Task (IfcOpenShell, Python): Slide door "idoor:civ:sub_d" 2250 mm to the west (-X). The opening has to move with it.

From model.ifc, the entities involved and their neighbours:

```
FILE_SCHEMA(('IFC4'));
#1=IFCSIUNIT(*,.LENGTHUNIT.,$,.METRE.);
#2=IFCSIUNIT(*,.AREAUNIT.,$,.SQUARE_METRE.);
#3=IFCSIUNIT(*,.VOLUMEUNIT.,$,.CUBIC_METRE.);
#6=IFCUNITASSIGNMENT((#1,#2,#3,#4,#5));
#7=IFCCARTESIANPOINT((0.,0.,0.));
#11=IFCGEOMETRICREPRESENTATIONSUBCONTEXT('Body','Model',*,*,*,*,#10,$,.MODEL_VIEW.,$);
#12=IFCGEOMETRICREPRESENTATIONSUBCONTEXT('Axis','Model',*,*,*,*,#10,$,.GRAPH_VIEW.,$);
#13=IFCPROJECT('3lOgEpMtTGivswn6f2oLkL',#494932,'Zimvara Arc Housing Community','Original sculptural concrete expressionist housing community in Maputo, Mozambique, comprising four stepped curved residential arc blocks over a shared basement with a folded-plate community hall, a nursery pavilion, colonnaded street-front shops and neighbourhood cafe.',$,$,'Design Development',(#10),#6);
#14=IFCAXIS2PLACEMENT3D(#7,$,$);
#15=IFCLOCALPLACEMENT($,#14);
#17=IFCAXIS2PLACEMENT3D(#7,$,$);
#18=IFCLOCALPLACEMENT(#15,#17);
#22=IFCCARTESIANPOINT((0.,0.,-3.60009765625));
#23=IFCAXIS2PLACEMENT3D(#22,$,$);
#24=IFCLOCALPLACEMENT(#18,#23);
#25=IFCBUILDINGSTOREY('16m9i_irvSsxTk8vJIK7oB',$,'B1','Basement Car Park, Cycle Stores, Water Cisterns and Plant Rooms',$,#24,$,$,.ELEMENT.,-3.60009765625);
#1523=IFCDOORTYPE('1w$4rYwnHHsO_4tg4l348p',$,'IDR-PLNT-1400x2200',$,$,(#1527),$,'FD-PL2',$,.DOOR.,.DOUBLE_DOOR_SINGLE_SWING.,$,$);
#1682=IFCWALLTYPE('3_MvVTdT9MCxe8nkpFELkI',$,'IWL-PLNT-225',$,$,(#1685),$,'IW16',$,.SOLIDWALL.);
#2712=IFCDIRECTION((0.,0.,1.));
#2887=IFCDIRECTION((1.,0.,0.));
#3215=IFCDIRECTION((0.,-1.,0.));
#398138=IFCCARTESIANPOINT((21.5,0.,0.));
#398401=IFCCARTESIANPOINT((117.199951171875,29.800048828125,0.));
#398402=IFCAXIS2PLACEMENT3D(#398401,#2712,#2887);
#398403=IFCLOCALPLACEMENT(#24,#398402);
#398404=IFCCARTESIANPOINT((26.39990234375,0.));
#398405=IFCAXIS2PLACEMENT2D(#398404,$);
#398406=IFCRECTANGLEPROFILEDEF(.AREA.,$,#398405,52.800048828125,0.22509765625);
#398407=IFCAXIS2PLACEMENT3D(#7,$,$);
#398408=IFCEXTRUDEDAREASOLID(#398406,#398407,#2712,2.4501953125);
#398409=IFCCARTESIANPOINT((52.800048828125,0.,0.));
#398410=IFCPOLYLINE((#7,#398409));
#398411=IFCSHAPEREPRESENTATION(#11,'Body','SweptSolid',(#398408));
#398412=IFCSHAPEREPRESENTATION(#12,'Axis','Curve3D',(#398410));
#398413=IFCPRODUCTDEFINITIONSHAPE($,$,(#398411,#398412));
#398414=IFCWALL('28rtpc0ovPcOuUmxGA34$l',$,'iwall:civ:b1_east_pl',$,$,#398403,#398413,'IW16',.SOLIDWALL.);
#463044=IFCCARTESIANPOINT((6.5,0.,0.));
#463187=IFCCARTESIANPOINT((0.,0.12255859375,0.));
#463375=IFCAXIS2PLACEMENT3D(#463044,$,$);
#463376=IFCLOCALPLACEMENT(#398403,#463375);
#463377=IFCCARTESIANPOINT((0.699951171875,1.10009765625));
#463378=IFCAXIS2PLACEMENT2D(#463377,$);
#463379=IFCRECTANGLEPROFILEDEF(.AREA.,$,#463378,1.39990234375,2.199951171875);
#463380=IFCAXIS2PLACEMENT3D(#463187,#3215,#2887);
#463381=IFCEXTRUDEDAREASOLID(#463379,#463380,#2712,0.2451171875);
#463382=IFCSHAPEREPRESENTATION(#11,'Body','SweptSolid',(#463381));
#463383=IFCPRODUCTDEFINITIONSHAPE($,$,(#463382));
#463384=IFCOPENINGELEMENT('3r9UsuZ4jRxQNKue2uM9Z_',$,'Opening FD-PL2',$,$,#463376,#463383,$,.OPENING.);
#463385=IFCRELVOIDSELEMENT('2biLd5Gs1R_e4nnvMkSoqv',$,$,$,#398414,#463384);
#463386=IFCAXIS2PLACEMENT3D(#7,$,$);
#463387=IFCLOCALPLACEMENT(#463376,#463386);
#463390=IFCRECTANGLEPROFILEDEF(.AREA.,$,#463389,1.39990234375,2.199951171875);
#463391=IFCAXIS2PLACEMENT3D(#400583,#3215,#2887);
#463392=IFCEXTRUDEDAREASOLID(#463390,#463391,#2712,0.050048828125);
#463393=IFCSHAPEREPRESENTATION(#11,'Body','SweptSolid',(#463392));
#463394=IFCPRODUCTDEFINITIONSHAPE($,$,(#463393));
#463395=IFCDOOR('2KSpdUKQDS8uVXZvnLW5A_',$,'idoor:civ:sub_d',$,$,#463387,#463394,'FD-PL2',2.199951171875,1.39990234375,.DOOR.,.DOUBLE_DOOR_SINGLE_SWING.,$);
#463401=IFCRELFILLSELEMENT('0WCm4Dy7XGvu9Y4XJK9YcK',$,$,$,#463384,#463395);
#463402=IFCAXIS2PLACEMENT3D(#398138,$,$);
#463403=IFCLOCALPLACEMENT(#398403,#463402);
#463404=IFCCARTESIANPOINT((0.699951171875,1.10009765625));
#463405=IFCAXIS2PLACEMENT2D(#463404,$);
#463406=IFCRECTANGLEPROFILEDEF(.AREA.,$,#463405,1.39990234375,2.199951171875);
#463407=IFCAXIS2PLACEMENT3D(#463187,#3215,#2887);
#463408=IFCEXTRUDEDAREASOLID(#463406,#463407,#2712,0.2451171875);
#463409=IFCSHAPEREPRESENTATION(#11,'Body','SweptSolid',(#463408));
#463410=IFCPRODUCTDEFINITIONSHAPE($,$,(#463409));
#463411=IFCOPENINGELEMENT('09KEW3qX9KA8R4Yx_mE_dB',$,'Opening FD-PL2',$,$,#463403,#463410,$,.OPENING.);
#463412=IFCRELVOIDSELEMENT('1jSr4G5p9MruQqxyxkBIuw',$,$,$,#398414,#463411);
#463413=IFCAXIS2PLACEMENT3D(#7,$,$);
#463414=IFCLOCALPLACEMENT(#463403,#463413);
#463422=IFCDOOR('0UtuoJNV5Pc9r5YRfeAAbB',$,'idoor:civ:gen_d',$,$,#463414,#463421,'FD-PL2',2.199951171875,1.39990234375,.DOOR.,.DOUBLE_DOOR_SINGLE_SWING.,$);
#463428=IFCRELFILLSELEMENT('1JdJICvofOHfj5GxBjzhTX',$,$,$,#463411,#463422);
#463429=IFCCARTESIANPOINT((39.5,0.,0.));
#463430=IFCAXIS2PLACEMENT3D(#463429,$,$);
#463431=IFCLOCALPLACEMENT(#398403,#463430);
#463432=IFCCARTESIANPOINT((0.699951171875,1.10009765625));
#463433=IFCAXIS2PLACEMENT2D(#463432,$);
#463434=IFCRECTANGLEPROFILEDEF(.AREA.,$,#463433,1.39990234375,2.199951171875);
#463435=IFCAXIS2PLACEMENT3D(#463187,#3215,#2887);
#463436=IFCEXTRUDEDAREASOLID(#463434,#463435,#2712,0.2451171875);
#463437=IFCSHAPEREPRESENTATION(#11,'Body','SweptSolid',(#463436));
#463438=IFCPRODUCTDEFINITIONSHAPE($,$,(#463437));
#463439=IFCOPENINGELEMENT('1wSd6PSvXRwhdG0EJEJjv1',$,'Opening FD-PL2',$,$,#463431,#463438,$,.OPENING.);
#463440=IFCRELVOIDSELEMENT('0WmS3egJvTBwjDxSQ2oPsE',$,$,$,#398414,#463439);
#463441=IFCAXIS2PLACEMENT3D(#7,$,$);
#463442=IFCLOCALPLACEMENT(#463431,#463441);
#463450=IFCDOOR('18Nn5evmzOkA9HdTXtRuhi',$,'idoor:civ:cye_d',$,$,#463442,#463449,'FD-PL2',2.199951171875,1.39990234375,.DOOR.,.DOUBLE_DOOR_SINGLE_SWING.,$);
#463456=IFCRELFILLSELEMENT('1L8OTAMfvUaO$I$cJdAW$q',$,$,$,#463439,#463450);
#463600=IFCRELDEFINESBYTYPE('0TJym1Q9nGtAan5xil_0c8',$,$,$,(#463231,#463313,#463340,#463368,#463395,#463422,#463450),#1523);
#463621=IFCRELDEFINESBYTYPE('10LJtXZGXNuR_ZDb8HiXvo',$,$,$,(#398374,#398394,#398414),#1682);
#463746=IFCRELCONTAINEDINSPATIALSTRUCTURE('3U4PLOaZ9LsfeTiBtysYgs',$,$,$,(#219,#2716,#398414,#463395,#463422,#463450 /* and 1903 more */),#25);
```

```python
import ifcopenshell
import ifcopenshell.api.geometry
import ifcopenshell.util.placement
import ifcopenshell.util.unit

model = ifcopenshell.open("model.ifc")
unit_scale = ifcopenshell.util.unit.calculate_unit_scale(model)

door = model.by_guid("2KSpdUKQDS8uVXZvnLW5A_")
opening = door.FillsVoids[0].RelatingOpeningElement
wall = opening.VoidsElements[0].RelatingBuildingElement

wall_matrix = ifcopenshell.util.placement.get_local_placement(wall.ObjectPlacement)
shift = wall_matrix[:3, 0] * -2.25 / unit_scale
before = ifcopenshell.util.placement.get_local_placement(door.ObjectPlacement)[:3, 3].copy()

# The door is placed relative to its opening, so it follows when the opening moves.
matrix = ifcopenshell.util.placement.get_local_placement(opening.ObjectPlacement)
matrix[:3, 3] += shift
ifcopenshell.api.geometry.edit_object_placement(
    model, product=opening, matrix=matrix, is_si=False, should_transform_children=True
)

after = ifcopenshell.util.placement.get_local_placement(door.ObjectPlacement)[:3, 3]
print("door moved by", (after - before).round(3) + 0.0)

model.write("model_rev.ifc")
```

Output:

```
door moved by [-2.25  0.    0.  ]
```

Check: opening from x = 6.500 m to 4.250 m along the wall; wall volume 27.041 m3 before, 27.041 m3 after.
